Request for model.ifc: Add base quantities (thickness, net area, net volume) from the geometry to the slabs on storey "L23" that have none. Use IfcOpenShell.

First a look at what the model holds.

```python
import ifcopenshell
import ifcopenshell.util.element
import ifcopenshell.util.unit

model = ifcopenshell.open("model.ifc")
print(model.schema)
for unit_type in ("LENGTHUNIT", "AREAUNIT", "VOLUMEUNIT"):
    print(unit_type, ifcopenshell.util.unit.calculate_unit_scale(model, unit_type))
storey = next(s for s in model.by_type("IfcBuildingStorey") if s.Name == "L23")
slabs = [e for e in ifcopenshell.util.element.get_decomposition(storey) if e.is_a("IfcSlab")]
for e in sorted(slabs, key=lambda e: e.id()):
    print(e.id(), e.is_a(), e.Name, list(ifcopenshell.util.element.get_psets(e, qtos_only=True)), sep=" | ")
```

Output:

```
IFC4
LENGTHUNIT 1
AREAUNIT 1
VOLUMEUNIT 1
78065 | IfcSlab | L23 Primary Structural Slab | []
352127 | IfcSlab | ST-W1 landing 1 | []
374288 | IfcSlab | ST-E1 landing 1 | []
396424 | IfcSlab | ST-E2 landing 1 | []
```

```python
import ifcopenshell
import ifcopenshell.api.pset
import ifcopenshell.geom
import ifcopenshell.util.element
import ifcopenshell.util.shape
import ifcopenshell.util.unit

model = ifcopenshell.open("model.ifc")
unit_scale = ifcopenshell.util.unit.calculate_unit_scale(model)
area_scale = ifcopenshell.util.unit.calculate_unit_scale(model, "AREAUNIT")
volume_scale = ifcopenshell.util.unit.calculate_unit_scale(model, "VOLUMEUNIT")
settings = ifcopenshell.geom.settings()

storey = next(s for s in model.by_type("IfcBuildingStorey") if s.Name == "L23")
slabs = [e for e in ifcopenshell.util.element.get_decomposition(storey) if e.is_a("IfcSlab")]

for e in sorted(slabs, key=lambda e: e.id()):
    if ifcopenshell.util.element.get_psets(e, qtos_only=True, should_inherit=False):
        continue
    # Geometry comes back in metres, in the element's own axes.
    shape = ifcopenshell.geom.create_shape(settings, e)
    values = {
        "Width": ifcopenshell.util.shape.get_z(shape.geometry) / unit_scale,
        "NetArea": ifcopenshell.util.shape.get_footprint_area(shape.geometry) / area_scale,
        "NetVolume": ifcopenshell.util.shape.get_volume(shape.geometry) / volume_scale,
    }
    qto = ifcopenshell.api.pset.add_qto(model, product=e, name="Qto_SlabBaseQuantities")
    ifcopenshell.api.pset.edit_qto(model, qto=qto, properties=values)
    print(e.id(), {k: round(v, 3) for k, v in values.items()})

model.write("model-out.ifc")
```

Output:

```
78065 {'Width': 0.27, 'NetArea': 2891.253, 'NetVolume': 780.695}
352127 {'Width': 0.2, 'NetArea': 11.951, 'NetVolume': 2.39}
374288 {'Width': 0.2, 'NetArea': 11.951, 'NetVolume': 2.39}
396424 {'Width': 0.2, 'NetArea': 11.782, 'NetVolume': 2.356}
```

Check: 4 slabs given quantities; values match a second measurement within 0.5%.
